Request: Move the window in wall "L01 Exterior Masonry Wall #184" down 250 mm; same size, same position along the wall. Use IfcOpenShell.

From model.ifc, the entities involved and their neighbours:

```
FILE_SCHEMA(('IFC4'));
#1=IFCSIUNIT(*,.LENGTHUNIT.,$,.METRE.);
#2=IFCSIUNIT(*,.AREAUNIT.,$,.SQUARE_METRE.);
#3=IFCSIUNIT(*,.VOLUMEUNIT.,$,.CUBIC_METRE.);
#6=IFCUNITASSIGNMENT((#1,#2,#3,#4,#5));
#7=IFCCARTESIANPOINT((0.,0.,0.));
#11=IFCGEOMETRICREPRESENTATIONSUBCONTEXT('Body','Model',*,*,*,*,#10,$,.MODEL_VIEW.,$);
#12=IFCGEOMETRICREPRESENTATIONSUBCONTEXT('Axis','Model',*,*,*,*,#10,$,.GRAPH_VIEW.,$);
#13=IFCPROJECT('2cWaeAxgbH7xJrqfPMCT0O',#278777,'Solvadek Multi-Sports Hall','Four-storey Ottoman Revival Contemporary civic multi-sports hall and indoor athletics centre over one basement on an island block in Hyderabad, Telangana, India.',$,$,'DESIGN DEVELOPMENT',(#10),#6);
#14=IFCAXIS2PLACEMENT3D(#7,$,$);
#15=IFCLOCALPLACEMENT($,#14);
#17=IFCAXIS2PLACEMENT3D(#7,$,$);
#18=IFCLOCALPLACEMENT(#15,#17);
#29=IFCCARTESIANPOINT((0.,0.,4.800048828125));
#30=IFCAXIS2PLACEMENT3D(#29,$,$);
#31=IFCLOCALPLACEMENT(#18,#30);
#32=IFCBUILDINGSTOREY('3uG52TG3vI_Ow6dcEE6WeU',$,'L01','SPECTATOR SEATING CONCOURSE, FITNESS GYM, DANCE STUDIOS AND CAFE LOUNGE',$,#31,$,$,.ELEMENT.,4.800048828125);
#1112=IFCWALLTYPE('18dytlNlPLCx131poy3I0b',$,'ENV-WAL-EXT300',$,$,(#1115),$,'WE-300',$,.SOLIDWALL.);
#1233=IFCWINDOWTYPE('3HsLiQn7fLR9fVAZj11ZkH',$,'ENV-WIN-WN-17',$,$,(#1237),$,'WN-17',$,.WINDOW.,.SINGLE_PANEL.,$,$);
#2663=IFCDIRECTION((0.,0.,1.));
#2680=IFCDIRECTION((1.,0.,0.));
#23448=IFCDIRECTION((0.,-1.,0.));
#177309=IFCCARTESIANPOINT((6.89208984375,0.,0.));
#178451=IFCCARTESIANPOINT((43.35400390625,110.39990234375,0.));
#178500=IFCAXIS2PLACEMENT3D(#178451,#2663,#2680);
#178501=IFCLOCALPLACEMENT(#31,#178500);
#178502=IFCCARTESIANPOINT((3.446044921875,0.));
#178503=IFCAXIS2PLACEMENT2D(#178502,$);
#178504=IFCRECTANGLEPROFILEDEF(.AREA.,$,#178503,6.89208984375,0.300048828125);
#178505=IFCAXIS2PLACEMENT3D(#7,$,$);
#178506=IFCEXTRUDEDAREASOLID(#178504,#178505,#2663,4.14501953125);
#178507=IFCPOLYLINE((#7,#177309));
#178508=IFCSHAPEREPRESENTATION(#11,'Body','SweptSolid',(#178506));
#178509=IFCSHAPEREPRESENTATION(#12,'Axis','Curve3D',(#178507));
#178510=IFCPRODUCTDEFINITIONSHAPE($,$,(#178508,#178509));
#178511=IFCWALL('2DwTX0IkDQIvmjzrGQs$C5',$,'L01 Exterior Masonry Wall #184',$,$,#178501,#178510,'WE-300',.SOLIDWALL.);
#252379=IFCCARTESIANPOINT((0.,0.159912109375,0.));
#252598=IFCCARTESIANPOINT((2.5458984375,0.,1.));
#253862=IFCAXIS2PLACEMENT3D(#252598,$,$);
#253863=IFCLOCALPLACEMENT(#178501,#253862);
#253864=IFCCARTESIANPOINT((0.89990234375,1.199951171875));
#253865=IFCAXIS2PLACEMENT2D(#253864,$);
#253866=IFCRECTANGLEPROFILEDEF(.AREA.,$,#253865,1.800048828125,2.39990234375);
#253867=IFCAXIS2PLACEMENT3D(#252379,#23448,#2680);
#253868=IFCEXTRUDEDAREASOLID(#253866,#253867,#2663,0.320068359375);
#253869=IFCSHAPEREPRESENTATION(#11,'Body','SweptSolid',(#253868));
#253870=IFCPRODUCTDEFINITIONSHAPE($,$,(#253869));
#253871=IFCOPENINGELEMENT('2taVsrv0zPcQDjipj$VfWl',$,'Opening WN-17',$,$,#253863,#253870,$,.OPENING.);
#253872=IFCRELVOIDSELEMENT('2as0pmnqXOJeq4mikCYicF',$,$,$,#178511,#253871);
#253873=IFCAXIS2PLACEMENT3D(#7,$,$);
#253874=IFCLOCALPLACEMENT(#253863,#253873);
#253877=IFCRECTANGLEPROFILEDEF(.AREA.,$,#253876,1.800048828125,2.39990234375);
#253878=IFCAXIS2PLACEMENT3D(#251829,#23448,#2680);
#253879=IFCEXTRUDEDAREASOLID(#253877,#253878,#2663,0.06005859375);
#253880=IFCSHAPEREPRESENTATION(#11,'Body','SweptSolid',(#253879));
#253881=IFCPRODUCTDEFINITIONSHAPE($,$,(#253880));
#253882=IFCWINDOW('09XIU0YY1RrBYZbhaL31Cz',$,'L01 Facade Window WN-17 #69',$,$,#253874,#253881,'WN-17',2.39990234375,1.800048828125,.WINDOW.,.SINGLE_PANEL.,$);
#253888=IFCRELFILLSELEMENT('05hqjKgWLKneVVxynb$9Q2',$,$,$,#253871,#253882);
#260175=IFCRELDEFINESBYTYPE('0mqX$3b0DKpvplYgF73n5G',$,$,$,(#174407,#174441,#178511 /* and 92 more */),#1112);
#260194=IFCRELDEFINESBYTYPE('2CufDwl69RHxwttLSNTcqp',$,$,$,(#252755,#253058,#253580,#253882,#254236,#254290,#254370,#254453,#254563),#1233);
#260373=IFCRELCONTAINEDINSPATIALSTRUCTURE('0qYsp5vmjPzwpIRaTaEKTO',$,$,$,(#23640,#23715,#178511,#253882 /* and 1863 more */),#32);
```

```python
import numpy as np
import ifcopenshell
import ifcopenshell.api.geometry
import ifcopenshell.util.placement
import ifcopenshell.util.unit

model = ifcopenshell.open("model.ifc")
unit_scale = ifcopenshell.util.unit.calculate_unit_scale(model)

window = model.by_guid("09XIU0YY1RrBYZbhaL31Cz")
opening = window.FillsVoids[0].RelatingOpeningElement
dz = -0.25

shift = np.array([0.0, 0.0, dz])
# The window is placed relative to its opening, so it follows when the opening moves.
matrix = ifcopenshell.util.placement.get_local_placement(opening.ObjectPlacement)
matrix[:3, 3] += shift
ifcopenshell.api.geometry.edit_object_placement(
    model, product=opening, matrix=matrix, is_si=False, should_transform_children=True
)

print(f"moved by {dz * unit_scale:+.3f} m")

model.write("model_edited.ifc")
```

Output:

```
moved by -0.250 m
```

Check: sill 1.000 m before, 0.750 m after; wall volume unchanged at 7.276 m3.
